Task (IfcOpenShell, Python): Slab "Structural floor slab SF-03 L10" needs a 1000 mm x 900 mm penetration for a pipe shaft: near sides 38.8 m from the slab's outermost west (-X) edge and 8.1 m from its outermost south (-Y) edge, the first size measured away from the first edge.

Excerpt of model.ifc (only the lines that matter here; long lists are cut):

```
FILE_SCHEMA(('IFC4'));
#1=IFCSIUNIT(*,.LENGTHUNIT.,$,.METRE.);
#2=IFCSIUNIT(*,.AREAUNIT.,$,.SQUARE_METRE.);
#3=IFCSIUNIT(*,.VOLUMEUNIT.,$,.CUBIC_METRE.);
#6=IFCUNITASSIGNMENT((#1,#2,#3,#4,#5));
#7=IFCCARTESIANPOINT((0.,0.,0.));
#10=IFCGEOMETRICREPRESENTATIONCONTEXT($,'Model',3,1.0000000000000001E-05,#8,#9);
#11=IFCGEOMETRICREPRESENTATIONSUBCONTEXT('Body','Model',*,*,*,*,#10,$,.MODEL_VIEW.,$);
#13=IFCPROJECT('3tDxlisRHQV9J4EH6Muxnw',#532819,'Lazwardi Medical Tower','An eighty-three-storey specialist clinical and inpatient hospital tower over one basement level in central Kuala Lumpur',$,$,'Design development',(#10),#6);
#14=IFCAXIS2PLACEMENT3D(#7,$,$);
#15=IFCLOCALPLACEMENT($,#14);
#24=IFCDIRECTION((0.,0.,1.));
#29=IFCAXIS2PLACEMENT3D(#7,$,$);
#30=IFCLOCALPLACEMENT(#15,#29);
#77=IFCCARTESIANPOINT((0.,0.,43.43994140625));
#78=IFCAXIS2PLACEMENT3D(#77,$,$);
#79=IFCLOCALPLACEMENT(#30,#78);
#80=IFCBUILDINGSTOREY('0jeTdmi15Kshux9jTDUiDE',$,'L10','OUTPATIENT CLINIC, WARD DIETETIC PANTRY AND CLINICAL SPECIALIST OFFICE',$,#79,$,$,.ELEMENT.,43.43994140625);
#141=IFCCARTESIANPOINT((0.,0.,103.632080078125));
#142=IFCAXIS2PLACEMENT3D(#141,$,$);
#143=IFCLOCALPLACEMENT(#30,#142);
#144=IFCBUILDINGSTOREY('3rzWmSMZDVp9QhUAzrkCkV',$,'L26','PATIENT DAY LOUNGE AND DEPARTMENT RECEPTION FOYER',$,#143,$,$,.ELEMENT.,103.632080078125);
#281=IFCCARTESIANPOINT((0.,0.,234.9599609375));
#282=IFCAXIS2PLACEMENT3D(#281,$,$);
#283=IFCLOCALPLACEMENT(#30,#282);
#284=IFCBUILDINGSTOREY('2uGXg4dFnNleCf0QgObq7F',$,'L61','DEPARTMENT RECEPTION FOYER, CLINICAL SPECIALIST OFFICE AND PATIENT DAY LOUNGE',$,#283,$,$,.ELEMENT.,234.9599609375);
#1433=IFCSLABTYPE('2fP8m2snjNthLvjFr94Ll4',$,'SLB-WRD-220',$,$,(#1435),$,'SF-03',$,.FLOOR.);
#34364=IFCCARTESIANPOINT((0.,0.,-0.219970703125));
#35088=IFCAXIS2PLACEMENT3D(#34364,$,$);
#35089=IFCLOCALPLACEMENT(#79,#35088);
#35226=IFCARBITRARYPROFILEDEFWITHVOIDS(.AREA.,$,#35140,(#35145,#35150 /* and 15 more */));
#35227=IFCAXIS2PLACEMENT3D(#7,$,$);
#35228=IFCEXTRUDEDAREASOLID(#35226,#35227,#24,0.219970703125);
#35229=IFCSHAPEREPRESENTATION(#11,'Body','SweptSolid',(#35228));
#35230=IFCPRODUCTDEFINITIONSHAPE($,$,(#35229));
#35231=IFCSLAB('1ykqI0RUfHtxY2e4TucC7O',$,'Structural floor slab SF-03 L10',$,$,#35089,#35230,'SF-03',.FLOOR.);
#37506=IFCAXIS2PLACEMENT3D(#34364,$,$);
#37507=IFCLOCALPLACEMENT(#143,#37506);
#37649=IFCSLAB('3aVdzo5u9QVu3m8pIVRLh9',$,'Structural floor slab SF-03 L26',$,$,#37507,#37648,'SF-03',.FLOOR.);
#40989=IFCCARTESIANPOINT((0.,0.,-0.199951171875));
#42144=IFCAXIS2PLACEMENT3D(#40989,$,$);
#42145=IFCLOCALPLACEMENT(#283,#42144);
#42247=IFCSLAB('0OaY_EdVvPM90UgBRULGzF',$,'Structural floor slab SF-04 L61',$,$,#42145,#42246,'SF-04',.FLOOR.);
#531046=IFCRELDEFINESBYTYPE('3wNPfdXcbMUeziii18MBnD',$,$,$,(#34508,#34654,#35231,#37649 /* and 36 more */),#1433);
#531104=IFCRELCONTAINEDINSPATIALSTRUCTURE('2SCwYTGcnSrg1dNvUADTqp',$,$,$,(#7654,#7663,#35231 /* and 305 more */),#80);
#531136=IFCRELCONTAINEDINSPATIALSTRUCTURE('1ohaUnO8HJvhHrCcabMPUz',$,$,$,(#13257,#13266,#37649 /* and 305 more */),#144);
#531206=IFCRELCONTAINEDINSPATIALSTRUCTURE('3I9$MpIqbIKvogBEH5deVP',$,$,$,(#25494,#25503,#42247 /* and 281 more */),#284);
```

```python
import numpy as np
import ifcopenshell
import ifcopenshell.api.feature
import ifcopenshell.api.geometry
import ifcopenshell.api.root
import ifcopenshell.geom
import ifcopenshell.util.placement
import ifcopenshell.util.representation
import ifcopenshell.util.shape
import ifcopenshell.util.unit

model = ifcopenshell.open("model.ifc")
unit_scale = ifcopenshell.util.unit.calculate_unit_scale(model)
settings = ifcopenshell.geom.settings()


def volume(element):
    """Net volume in cubic metres, openings subtracted."""
    shape = ifcopenshell.geom.create_shape(settings, element)
    return ifcopenshell.util.shape.get_volume(shape.geometry)


slab = model.by_id(35231)
before = volume(slab)

# Extent in the slab's own axes, in metres. The edges named are its -X and -Y sides.
slab_shape = ifcopenshell.geom.create_shape(settings, slab)
vertices = ifcopenshell.util.shape.get_vertices(slab_shape.geometry)
x_min, y_min, bottom = vertices.min(axis=0)
top = vertices[:, 2].max()

opening = ifcopenshell.api.root.create_entity(model, ifc_class="IfcOpeningElement", name="Pipe shaft opening", predefined_type="OPENING")
context = ifcopenshell.util.representation.get_context(model, "Model", "Body", "MODEL_VIEW")
width, depth = 1, 0.9
outline = [(0.0, 0.0), (width, 0.0), (width, depth), (0.0, depth), (0.0, 0.0)]
# Overshoot both faces by 50 mm so the cut is clean.
shape = ifcopenshell.api.geometry.add_slab_representation(
    model, context=context, depth=top - bottom + 0.1, polyline=outline
)
ifcopenshell.api.geometry.assign_representation(model, product=opening, representation=shape)

matrix = ifcopenshell.util.placement.get_local_placement(slab.ObjectPlacement)
matrix[:, 3] = matrix @ np.append(np.array([x_min + 38.8, y_min + 8.1, bottom - 0.05]) / unit_scale, 1.0)
ifcopenshell.api.geometry.edit_object_placement(model, product=opening, matrix=matrix, is_si=False)
ifcopenshell.api.feature.add_feature(model, feature=opening, element=slab)

after = volume(slab)

print(f"slab volume {before:.3f} -> {after:.3f} m3")

model.write("model_updated.ifc")
```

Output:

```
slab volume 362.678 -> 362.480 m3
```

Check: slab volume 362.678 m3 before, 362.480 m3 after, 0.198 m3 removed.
